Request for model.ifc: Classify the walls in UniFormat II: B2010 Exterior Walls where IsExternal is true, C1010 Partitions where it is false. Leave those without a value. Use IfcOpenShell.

First a look at what the model holds.

```python
import ifcopenshell
import ifcopenshell.util.element

model = ifcopenshell.open("model.ifc")
print(model.schema)
print("classifications:", [c.Name for c in model.by_type("IfcClassification")])
values = [ifcopenshell.util.element.get_pset(e, "Pset_WallCommon", "IsExternal") for e in model.by_type("IfcWall")]
for value in (True, False, None):
    print("IsExternal", value, values.count(value))
```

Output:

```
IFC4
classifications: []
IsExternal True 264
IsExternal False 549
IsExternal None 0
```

```python
import ifcopenshell
import ifcopenshell.api.classification
import ifcopenshell.util.element

model = ifcopenshell.open("model.ifc")

system = ifcopenshell.api.classification.add_classification(model, classification="UniFormat II")

walls = model.by_type("IfcWall")
external = {e: ifcopenshell.util.element.get_pset(e, "Pset_WallCommon", "IsExternal") for e in walls}
for flag, code, name in ((True, "B2010", "Exterior Walls"), (False, "C1010", "Partitions")):
    products = [e for e in walls if external[e] is flag]
    ifcopenshell.api.classification.add_reference(
        model, products=products, classification=system, identification=code, name=name
    )
    print(code, len(products))

model.write("model_edited.ifc")
```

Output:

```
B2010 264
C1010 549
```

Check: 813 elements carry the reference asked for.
